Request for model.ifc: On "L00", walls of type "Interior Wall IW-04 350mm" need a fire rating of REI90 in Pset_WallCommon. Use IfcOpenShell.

First a look at what the model holds.

```python
import ifcopenshell
import ifcopenshell.util.element

model = ifcopenshell.open("model.ifc")
print(model.schema)
storey = next(s for s in model.by_type("IfcBuildingStorey") if s.Name == "L00")
walls = [e for e in ifcopenshell.util.element.get_decomposition(storey) if e.is_a("IfcWall")]
seen = {}
for e in walls:
    element_type = ifcopenshell.util.element.get_type(e)
    key = (element_type.Name if element_type != e and element_type else None, ifcopenshell.util.element.get_pset(e, "Pset_WallCommon", "FireRating"))
    seen[key] = seen.get(key, 0) + 1
for (name, value), count in sorted(seen.items(), key=str):
    print(count, "x", name, "|", value)
```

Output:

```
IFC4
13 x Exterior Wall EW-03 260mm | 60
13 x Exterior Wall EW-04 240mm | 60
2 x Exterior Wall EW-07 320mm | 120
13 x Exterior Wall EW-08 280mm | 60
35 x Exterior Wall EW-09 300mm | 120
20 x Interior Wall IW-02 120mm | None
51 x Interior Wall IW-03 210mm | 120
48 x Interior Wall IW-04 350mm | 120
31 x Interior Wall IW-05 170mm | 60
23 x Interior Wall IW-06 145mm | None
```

```python
import ifcopenshell
import ifcopenshell.api.pset
import ifcopenshell.util.element

model = ifcopenshell.open("model.ifc")

storey = next(s for s in model.by_type("IfcBuildingStorey") if s.Name == "L00")
walls = [e for e in ifcopenshell.util.element.get_decomposition(storey) if e.is_a("IfcWall")]

count = 0
for e in walls:
    element_type = ifcopenshell.util.element.get_type(e)
    if element_type in (None, e) or element_type.Name != "Interior Wall IW-04 350mm":
        continue
    # add_pset returns the element's existing set when there is one.
    pset = ifcopenshell.api.pset.add_pset(model, product=e, name="Pset_WallCommon")
    ifcopenshell.api.pset.edit_pset(model, pset=pset, properties={"FireRating": "REI90"})
    count += 1

print(count, "walls updated")

model.write("model_updated.ifc")
```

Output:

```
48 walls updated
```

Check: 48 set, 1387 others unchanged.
